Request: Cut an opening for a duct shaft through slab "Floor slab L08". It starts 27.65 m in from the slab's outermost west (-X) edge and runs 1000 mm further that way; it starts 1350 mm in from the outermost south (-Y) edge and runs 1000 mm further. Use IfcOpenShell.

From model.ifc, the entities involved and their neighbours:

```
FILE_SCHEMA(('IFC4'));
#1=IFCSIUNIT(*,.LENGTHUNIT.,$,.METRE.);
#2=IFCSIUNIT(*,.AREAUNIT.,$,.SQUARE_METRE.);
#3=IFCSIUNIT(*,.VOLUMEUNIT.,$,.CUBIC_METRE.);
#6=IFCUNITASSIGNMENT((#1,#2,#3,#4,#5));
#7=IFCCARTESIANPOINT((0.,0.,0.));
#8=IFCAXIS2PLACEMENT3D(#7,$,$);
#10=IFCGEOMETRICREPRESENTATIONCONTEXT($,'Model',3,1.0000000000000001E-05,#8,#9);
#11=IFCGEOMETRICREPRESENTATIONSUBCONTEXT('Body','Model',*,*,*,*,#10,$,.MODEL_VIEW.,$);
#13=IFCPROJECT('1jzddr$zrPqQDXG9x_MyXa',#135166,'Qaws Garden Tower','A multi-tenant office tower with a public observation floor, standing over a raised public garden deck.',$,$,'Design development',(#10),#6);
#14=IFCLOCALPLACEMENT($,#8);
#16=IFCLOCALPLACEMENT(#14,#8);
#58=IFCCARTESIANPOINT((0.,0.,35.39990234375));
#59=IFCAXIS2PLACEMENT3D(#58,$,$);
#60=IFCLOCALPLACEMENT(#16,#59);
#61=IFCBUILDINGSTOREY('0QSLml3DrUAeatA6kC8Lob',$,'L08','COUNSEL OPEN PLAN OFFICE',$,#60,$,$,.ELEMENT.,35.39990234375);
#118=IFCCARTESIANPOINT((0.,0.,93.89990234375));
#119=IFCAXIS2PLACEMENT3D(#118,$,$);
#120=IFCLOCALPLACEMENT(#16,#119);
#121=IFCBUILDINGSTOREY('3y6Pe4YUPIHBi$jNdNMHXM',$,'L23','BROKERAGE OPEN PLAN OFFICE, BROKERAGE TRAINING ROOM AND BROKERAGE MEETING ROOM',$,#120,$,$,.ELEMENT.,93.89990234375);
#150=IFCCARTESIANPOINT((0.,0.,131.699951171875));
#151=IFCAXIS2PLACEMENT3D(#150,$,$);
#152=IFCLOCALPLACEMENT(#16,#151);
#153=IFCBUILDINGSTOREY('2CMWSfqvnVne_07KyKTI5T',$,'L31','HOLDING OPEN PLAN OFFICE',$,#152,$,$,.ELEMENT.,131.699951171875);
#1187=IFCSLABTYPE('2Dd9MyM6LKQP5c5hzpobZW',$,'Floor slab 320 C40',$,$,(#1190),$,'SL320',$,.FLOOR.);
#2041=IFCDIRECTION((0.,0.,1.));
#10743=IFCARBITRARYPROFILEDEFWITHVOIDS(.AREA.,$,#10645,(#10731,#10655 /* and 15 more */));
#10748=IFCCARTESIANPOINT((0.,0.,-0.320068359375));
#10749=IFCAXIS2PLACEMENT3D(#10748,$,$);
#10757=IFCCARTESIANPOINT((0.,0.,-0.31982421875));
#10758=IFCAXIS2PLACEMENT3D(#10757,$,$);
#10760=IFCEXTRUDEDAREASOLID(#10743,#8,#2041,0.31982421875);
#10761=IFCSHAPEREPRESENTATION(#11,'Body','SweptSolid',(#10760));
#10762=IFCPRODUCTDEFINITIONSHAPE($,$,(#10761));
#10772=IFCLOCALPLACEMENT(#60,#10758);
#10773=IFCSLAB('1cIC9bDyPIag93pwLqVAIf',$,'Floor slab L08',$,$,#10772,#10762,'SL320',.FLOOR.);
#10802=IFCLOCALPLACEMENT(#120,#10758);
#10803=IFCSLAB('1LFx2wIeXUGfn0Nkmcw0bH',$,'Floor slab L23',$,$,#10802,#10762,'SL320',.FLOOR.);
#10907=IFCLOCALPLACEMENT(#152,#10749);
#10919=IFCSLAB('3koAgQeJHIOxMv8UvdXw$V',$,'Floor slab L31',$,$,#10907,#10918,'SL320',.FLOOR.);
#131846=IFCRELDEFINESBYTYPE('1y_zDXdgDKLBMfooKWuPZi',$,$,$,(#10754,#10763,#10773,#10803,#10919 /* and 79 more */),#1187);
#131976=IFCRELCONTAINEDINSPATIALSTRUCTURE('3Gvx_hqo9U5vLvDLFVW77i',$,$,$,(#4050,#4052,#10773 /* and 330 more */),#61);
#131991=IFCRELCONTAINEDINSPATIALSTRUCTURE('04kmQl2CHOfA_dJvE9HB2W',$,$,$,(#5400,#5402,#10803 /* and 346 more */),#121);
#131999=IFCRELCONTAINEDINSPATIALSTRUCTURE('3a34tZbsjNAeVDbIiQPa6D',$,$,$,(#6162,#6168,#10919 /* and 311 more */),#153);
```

```python
import numpy as np
import ifcopenshell
import ifcopenshell.api.feature
import ifcopenshell.api.geometry
import ifcopenshell.api.root
import ifcopenshell.geom
import ifcopenshell.util.placement
import ifcopenshell.util.representation
import ifcopenshell.util.shape
import ifcopenshell.util.unit

model = ifcopenshell.open("model.ifc")
unit_scale = ifcopenshell.util.unit.calculate_unit_scale(model)
settings = ifcopenshell.geom.settings()


def volume(element):
    """Net volume in cubic metres, openings subtracted."""
    shape = ifcopenshell.geom.create_shape(settings, element)
    return ifcopenshell.util.shape.get_volume(shape.geometry)


slab = model.by_guid("1cIC9bDyPIag93pwLqVAIf")
before = volume(slab)

# Extent in the slab's own axes, in metres. The edges named are its -X and -Y sides.
slab_shape = ifcopenshell.geom.create_shape(settings, slab)
vertices = ifcopenshell.util.shape.get_vertices(slab_shape.geometry)
x_min, y_min, bottom = vertices.min(axis=0)
top = vertices[:, 2].max()

opening = ifcopenshell.api.root.create_entity(model, ifc_class="IfcOpeningElement", name="Duct shaft opening", predefined_type="OPENING")
context = ifcopenshell.util.representation.get_context(model, "Model", "Body", "MODEL_VIEW")
width, depth = 1, 1
outline = [(0.0, 0.0), (width, 0.0), (width, depth), (0.0, depth), (0.0, 0.0)]
# Overshoot both faces by 50 mm so the cut is clean.
shape = ifcopenshell.api.geometry.add_slab_representation(
    model, context=context, depth=top - bottom + 0.1, polyline=outline
)
ifcopenshell.api.geometry.assign_representation(model, product=opening, representation=shape)

matrix = ifcopenshell.util.placement.get_local_placement(slab.ObjectPlacement)
matrix[:, 3] = matrix @ np.append(np.array([x_min + 27.65, y_min + 1.35, bottom - 0.05]) / unit_scale, 1.0)
ifcopenshell.api.geometry.edit_object_placement(model, product=opening, matrix=matrix, is_si=False)
ifcopenshell.api.feature.add_feature(model, feature=opening, element=slab)

after = volume(slab)

print(f"slab volume {before:.3f} -> {after:.3f} m3")

model.write("model-out.ifc")
```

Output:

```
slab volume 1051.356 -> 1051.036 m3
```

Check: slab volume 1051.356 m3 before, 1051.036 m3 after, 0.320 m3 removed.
